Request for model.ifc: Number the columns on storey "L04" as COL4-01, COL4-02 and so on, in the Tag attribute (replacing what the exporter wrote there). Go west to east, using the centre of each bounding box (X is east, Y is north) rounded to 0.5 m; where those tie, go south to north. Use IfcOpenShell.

First a look at what the model holds.

```python
import ifcopenshell
import ifcopenshell.util.element
import ifcopenshell.util.placement

model = ifcopenshell.open("model.ifc")
print(model.schema)
storey = next(s for s in model.by_type("IfcBuildingStorey") if s.Name == "L04")
columns = [e for e in ifcopenshell.util.element.get_decomposition(storey) if e.is_a("IfcColumn")]
for e in sorted(columns, key=lambda e: e.id()):
    origin = ifcopenshell.util.placement.get_local_placement(e.ObjectPlacement)[:3, 3]
    print(e.id(), e.Tag, e.Name, origin.round(2) + 0.0, sep=" | ")
```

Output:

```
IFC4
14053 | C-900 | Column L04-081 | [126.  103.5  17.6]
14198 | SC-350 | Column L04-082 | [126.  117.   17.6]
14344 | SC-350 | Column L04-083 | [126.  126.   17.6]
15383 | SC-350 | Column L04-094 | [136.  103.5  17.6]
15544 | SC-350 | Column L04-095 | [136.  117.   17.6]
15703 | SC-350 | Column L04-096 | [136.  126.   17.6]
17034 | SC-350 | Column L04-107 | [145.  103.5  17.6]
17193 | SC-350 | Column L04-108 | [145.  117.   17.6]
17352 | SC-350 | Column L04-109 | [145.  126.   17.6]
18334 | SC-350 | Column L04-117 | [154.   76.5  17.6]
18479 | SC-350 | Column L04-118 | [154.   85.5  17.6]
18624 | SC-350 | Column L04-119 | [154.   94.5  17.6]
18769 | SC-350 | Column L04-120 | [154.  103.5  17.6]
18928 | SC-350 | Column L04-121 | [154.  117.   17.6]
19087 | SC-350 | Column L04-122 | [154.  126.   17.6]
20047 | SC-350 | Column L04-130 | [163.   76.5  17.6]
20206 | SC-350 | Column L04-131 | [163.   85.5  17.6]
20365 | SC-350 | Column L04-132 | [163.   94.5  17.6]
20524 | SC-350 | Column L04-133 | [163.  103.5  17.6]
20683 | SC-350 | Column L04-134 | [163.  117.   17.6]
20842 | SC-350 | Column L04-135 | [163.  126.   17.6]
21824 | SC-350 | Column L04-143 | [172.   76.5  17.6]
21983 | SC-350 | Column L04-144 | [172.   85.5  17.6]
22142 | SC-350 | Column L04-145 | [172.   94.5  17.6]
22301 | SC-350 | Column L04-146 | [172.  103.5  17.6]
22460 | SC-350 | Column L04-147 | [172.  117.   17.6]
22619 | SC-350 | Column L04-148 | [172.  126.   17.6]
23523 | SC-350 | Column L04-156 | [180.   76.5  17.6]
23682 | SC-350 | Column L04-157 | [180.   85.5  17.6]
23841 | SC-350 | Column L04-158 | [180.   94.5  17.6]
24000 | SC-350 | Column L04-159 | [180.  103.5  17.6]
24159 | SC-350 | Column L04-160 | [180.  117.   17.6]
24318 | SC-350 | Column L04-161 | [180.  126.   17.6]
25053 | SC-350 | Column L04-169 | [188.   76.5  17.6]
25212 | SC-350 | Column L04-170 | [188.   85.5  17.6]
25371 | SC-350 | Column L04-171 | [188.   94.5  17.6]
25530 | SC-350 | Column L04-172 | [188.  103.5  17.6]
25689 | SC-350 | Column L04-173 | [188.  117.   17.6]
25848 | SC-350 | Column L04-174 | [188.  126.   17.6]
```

```python
import ifcopenshell
import ifcopenshell.geom
import ifcopenshell.util.element
import ifcopenshell.util.shape

model = ifcopenshell.open("model.ifc")
settings = ifcopenshell.geom.settings()
settings.set("use-world-coords", True)


def centre(element):
    shape = ifcopenshell.geom.create_shape(settings, element)
    return ifcopenshell.util.shape.get_bbox_centroid(shape.geometry)


storey = next(s for s in model.by_type("IfcBuildingStorey") if s.Name == "L04")
columns = [e for e in ifcopenshell.util.element.get_decomposition(storey) if e.is_a("IfcColumn")]

# Insertion points can sit at a corner or the storey origin, so sort by the geometry (in metres).
centres = {e: centre(e) for e in columns}
columns.sort(key=lambda e: (round(centres[e][0] / 0.5), centres[e][1]))

for i, e in enumerate(columns, start=1):
    number = f"COL4-{i:02d}"
    e.Tag = number
    print(e.id(), number)

model.write("model-out.ifc")
```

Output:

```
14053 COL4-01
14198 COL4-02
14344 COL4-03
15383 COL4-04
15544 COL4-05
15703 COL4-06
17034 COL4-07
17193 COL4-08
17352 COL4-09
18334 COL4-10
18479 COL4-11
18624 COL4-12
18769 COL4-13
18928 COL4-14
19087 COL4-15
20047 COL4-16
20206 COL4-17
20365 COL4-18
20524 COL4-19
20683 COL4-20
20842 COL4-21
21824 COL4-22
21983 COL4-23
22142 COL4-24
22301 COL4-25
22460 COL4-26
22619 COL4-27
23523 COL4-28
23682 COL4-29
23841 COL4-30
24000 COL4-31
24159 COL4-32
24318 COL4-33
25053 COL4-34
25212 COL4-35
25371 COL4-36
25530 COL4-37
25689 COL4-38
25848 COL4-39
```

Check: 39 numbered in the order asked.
